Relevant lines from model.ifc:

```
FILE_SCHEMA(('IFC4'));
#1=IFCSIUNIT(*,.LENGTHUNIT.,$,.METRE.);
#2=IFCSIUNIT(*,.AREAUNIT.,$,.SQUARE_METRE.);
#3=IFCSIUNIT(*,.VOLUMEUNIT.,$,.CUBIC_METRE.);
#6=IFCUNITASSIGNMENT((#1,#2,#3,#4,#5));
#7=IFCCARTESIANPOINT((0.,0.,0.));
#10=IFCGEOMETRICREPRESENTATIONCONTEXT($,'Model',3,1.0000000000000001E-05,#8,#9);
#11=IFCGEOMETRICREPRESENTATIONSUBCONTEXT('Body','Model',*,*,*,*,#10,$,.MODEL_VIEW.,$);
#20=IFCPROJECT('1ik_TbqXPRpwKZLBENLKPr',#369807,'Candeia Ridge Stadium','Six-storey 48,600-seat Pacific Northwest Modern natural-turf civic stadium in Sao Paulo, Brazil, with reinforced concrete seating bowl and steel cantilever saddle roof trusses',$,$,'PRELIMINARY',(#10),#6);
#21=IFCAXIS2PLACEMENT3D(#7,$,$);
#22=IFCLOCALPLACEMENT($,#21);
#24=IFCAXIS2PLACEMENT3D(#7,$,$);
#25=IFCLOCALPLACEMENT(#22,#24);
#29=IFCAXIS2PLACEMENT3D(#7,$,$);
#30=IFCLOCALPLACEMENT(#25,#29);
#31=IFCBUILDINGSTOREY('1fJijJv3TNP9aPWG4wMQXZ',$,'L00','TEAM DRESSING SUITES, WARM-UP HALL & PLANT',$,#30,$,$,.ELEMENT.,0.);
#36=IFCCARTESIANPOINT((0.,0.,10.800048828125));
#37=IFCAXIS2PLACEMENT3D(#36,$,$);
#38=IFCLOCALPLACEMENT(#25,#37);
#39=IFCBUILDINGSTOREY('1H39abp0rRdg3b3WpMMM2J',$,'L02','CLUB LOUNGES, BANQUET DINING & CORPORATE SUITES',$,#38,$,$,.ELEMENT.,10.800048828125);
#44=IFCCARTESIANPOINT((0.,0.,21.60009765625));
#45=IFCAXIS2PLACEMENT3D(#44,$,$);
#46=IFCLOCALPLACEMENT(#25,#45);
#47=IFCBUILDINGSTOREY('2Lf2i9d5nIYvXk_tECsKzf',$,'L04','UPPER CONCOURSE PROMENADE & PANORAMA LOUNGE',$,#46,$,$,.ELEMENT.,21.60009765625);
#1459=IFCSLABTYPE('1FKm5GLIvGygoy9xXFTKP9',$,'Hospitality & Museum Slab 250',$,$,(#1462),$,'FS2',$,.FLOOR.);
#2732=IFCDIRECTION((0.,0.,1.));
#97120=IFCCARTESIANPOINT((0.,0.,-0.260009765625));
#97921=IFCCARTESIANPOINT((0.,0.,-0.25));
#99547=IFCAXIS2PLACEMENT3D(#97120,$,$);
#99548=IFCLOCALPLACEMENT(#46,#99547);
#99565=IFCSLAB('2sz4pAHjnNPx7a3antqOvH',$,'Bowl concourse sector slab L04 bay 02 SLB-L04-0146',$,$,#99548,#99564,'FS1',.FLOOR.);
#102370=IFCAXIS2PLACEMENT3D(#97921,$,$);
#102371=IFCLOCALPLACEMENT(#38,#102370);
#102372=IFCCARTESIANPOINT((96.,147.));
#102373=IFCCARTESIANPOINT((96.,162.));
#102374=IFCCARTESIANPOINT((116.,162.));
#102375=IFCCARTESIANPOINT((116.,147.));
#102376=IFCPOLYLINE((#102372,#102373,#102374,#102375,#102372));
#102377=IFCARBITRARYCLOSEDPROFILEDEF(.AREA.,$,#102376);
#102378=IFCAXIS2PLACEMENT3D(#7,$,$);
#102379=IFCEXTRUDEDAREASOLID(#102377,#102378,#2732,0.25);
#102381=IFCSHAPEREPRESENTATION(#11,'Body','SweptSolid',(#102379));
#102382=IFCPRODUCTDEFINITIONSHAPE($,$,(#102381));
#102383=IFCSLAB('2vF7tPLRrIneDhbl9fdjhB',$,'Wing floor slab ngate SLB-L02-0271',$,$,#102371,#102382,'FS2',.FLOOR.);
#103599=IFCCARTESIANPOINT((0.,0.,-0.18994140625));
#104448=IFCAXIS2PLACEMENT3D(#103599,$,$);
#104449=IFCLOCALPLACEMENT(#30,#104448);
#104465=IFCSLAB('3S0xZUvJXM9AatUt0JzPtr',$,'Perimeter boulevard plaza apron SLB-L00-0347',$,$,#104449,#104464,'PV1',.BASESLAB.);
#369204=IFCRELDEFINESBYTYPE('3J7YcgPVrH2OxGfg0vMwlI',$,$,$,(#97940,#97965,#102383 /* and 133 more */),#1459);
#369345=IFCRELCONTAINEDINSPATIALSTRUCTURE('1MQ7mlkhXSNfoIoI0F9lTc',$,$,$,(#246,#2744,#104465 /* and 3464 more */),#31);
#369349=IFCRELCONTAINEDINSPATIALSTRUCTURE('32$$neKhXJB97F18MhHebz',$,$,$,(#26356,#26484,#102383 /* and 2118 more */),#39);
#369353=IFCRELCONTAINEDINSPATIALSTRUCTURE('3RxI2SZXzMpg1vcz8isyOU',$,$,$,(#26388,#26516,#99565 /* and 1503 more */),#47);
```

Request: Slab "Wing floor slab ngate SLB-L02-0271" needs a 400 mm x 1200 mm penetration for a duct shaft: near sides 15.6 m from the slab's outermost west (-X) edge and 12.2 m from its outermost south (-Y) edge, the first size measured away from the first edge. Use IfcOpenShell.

```python
import numpy as np
import ifcopenshell
import ifcopenshell.api.feature
import ifcopenshell.api.geometry
import ifcopenshell.api.root
import ifcopenshell.geom
import ifcopenshell.util.placement
import ifcopenshell.util.representation
import ifcopenshell.util.shape
import ifcopenshell.util.unit

model = ifcopenshell.open("model.ifc")
unit_scale = ifcopenshell.util.unit.calculate_unit_scale(model)
settings = ifcopenshell.geom.settings()


def volume(element):
    """Net volume in cubic metres, openings subtracted."""
    shape = ifcopenshell.geom.create_shape(settings, element)
    return ifcopenshell.util.shape.get_volume(shape.geometry)


slab = model.by_id(102383)
before = volume(slab)

# Extent in the slab's own axes, in metres. The edges named are its -X and -Y sides.
slab_shape = ifcopenshell.geom.create_shape(settings, slab)
vertices = ifcopenshell.util.shape.get_vertices(slab_shape.geometry)
x_min, y_min, bottom = vertices.min(axis=0)
top = vertices[:, 2].max()

opening = ifcopenshell.api.root.create_entity(model, ifc_class="IfcOpeningElement", name="Duct shaft opening", predefined_type="OPENING")
context = ifcopenshell.util.representation.get_context(model, "Model", "Body", "MODEL_VIEW")
width, depth = 0.4, 1.2
outline = [(0.0, 0.0), (width, 0.0), (width, depth), (0.0, depth), (0.0, 0.0)]
# Overshoot both faces by 50 mm so the cut is clean.
shape = ifcopenshell.api.geometry.add_slab_representation(
    model, context=context, depth=top - bottom + 0.1, polyline=outline
)
ifcopenshell.api.geometry.assign_representation(model, product=opening, representation=shape)

matrix = ifcopenshell.util.placement.get_local_placement(slab.ObjectPlacement)
matrix[:, 3] = matrix @ np.append(np.array([x_min + 15.6, y_min + 12.2, bottom - 0.05]) / unit_scale, 1.0)
ifcopenshell.api.geometry.edit_object_placement(model, product=opening, matrix=matrix, is_si=False)
ifcopenshell.api.feature.add_feature(model, feature=opening, element=slab)

after = volume(slab)

print(f"slab volume {before:.3f} -> {after:.3f} m3")

model.write("model-out.ifc")
```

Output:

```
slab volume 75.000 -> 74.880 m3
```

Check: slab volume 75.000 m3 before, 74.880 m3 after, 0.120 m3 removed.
